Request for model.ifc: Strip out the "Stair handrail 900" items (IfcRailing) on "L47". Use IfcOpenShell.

First a look at what the model holds.

```python
import ifcopenshell
import ifcopenshell.util.element

model = ifcopenshell.open("model.ifc")
print(model.schema)
storey = next(s for s in model.by_type("IfcBuildingStorey") if s.Name == "L47")
railings = [e for e in ifcopenshell.util.element.get_decomposition(storey) if e.is_a("IfcRailing")]
seen = {}
for e in railings:
    element_type = ifcopenshell.util.element.get_type(e)
    name = element_type.Name if element_type not in (None, e) else None
    seen[name] = seen.get(name, 0) + 1
for name, count in sorted(seen.items(), key=str):
    print(count, "x", name)
```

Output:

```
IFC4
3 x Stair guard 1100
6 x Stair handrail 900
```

```python
import ifcopenshell
import ifcopenshell.api.root
import ifcopenshell.util.element

model = ifcopenshell.open("model.ifc")

storey = next(s for s in model.by_type("IfcBuildingStorey") if s.Name == "L47")
railings = [e for e in ifcopenshell.util.element.get_decomposition(storey) if e.is_a("IfcRailing")]
targets = [e for e in railings if (t := ifcopenshell.util.element.get_type(e)) not in (None, e) and t.Name == "Stair handrail 900"]

for e in targets:
    ifcopenshell.api.root.remove_product(model, product=e)
print(len(targets), "removed")

model.write("model_edited.ifc")
```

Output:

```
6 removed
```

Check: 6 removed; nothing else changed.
